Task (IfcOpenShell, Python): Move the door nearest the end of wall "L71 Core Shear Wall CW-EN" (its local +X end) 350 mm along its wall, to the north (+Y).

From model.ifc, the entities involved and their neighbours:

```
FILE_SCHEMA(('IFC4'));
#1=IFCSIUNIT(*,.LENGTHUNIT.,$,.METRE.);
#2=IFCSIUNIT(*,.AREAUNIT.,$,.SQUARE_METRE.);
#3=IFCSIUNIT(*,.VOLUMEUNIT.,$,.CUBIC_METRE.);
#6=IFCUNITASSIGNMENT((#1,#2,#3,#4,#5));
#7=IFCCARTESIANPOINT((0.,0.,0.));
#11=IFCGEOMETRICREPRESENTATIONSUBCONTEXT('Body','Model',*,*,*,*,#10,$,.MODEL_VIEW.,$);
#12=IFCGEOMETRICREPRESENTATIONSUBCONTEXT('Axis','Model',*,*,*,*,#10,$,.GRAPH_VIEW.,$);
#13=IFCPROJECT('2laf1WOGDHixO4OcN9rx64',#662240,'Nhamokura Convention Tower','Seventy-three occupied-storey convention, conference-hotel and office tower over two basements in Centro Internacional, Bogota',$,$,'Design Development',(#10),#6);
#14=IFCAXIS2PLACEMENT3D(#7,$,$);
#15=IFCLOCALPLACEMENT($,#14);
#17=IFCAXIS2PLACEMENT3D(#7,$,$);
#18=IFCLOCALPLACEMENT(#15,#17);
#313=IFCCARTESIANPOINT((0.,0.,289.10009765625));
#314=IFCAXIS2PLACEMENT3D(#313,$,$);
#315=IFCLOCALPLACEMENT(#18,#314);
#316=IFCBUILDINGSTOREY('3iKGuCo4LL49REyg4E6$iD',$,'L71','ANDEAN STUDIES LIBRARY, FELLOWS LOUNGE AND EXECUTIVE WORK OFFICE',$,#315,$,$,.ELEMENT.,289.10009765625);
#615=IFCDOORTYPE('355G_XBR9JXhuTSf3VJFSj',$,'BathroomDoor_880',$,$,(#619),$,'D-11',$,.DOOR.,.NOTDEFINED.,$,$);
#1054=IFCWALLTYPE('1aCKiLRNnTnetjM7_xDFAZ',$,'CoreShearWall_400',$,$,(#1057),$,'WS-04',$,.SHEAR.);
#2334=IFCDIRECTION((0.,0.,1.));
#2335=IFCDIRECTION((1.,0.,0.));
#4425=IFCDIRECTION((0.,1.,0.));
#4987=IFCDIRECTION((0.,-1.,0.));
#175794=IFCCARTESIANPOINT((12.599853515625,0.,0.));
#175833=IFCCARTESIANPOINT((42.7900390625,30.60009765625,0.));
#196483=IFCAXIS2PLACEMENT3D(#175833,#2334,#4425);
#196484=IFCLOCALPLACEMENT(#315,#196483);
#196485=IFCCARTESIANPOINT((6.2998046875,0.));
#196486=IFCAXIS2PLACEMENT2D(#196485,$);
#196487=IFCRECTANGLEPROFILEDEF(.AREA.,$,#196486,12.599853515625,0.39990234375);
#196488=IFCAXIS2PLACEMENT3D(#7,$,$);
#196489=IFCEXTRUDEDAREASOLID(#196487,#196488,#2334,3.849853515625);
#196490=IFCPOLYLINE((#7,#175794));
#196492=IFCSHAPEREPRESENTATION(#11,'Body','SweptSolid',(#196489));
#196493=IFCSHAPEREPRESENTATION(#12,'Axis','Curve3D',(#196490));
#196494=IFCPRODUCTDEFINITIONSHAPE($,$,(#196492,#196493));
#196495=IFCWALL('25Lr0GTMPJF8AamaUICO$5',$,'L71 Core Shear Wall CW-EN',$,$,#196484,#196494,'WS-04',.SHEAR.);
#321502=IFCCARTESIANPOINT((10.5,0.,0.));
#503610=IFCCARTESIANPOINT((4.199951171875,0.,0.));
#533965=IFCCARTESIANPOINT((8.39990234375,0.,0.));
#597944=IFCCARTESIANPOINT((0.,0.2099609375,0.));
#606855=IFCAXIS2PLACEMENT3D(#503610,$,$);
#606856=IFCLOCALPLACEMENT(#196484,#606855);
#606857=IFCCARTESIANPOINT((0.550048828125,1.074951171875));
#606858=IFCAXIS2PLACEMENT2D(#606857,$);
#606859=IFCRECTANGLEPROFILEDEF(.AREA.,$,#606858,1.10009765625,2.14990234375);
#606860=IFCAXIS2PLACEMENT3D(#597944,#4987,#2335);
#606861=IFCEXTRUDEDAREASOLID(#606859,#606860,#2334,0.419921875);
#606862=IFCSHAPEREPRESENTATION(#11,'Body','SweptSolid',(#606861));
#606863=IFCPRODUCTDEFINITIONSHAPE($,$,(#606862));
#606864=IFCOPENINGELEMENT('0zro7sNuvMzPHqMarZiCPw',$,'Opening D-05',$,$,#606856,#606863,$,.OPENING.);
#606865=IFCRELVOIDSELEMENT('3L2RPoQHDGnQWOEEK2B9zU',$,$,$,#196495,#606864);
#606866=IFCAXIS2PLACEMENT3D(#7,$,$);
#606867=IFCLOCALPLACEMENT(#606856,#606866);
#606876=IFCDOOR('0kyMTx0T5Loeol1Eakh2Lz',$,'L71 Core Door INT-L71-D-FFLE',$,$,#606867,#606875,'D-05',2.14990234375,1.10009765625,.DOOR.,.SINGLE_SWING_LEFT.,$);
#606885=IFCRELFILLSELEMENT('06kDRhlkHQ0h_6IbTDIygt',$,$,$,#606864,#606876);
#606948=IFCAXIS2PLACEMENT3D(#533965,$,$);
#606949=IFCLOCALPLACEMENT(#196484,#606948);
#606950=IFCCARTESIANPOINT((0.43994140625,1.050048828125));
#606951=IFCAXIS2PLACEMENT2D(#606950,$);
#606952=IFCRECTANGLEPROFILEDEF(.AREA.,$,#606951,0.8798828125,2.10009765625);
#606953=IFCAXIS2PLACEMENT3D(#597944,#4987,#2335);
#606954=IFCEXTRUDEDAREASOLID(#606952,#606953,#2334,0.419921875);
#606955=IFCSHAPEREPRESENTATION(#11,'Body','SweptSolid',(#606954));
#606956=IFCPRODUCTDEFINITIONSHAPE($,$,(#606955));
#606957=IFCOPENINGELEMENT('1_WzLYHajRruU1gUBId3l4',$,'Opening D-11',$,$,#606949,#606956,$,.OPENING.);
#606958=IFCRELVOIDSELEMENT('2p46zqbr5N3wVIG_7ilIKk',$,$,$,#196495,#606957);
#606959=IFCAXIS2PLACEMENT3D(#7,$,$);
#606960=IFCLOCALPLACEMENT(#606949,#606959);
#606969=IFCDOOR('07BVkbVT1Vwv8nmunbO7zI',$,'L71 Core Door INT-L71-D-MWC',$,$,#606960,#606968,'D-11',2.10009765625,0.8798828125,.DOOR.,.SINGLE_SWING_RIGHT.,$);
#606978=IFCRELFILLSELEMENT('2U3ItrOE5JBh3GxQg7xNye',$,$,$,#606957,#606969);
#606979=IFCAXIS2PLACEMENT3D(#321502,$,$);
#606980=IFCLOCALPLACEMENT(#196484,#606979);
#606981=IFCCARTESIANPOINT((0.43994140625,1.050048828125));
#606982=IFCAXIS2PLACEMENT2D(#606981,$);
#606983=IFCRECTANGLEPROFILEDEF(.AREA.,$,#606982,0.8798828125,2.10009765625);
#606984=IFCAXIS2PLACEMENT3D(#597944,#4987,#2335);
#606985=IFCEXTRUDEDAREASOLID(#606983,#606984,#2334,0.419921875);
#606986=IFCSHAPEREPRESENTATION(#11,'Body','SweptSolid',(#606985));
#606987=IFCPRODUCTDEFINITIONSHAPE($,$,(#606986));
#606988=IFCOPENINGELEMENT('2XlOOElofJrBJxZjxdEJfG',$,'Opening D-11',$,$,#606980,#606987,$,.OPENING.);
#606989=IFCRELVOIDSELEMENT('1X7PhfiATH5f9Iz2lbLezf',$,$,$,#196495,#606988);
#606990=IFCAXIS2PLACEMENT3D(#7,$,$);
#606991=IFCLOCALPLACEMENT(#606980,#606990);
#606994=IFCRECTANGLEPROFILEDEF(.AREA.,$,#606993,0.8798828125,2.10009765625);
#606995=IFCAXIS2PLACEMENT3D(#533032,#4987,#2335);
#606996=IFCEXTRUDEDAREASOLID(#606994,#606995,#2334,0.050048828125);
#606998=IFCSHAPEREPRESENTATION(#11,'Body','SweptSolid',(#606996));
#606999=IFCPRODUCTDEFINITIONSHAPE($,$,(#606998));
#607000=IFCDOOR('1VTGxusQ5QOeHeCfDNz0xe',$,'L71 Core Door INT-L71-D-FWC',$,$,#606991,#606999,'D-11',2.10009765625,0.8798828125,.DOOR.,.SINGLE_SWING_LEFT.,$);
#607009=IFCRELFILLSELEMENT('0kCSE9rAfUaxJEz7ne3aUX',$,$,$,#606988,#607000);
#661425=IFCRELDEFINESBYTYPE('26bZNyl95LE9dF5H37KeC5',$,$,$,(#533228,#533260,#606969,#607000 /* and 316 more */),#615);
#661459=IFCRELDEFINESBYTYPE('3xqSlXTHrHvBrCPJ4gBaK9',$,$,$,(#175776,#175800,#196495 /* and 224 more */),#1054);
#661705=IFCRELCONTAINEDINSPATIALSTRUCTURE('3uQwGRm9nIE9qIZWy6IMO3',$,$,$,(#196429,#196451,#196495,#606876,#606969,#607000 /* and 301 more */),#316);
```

```python
import ifcopenshell
import ifcopenshell.api.geometry
import ifcopenshell.util.placement
import ifcopenshell.util.unit

model = ifcopenshell.open("model.ifc")
unit_scale = ifcopenshell.util.unit.calculate_unit_scale(model)

door = model.by_guid("1VTGxusQ5QOeHeCfDNz0xe")
opening = door.FillsVoids[0].RelatingOpeningElement
wall = opening.VoidsElements[0].RelatingBuildingElement

wall_matrix = ifcopenshell.util.placement.get_local_placement(wall.ObjectPlacement)
shift = wall_matrix[:3, 0] * 0.35 / unit_scale
before = ifcopenshell.util.placement.get_local_placement(door.ObjectPlacement)[:3, 3].copy()

# The door is placed relative to its opening, so it follows when the opening moves.
matrix = ifcopenshell.util.placement.get_local_placement(opening.ObjectPlacement)
matrix[:3, 3] += shift
ifcopenshell.api.geometry.edit_object_placement(
    model, product=opening, matrix=matrix, is_si=False, should_transform_children=True
)

after = ifcopenshell.util.placement.get_local_placement(door.ObjectPlacement)[:3, 3]
print("door moved by", (after - before).round(3) + 0.0)

model.write("model-out.ifc")
```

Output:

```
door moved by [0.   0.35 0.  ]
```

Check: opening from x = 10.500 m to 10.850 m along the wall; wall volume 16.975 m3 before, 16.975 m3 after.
